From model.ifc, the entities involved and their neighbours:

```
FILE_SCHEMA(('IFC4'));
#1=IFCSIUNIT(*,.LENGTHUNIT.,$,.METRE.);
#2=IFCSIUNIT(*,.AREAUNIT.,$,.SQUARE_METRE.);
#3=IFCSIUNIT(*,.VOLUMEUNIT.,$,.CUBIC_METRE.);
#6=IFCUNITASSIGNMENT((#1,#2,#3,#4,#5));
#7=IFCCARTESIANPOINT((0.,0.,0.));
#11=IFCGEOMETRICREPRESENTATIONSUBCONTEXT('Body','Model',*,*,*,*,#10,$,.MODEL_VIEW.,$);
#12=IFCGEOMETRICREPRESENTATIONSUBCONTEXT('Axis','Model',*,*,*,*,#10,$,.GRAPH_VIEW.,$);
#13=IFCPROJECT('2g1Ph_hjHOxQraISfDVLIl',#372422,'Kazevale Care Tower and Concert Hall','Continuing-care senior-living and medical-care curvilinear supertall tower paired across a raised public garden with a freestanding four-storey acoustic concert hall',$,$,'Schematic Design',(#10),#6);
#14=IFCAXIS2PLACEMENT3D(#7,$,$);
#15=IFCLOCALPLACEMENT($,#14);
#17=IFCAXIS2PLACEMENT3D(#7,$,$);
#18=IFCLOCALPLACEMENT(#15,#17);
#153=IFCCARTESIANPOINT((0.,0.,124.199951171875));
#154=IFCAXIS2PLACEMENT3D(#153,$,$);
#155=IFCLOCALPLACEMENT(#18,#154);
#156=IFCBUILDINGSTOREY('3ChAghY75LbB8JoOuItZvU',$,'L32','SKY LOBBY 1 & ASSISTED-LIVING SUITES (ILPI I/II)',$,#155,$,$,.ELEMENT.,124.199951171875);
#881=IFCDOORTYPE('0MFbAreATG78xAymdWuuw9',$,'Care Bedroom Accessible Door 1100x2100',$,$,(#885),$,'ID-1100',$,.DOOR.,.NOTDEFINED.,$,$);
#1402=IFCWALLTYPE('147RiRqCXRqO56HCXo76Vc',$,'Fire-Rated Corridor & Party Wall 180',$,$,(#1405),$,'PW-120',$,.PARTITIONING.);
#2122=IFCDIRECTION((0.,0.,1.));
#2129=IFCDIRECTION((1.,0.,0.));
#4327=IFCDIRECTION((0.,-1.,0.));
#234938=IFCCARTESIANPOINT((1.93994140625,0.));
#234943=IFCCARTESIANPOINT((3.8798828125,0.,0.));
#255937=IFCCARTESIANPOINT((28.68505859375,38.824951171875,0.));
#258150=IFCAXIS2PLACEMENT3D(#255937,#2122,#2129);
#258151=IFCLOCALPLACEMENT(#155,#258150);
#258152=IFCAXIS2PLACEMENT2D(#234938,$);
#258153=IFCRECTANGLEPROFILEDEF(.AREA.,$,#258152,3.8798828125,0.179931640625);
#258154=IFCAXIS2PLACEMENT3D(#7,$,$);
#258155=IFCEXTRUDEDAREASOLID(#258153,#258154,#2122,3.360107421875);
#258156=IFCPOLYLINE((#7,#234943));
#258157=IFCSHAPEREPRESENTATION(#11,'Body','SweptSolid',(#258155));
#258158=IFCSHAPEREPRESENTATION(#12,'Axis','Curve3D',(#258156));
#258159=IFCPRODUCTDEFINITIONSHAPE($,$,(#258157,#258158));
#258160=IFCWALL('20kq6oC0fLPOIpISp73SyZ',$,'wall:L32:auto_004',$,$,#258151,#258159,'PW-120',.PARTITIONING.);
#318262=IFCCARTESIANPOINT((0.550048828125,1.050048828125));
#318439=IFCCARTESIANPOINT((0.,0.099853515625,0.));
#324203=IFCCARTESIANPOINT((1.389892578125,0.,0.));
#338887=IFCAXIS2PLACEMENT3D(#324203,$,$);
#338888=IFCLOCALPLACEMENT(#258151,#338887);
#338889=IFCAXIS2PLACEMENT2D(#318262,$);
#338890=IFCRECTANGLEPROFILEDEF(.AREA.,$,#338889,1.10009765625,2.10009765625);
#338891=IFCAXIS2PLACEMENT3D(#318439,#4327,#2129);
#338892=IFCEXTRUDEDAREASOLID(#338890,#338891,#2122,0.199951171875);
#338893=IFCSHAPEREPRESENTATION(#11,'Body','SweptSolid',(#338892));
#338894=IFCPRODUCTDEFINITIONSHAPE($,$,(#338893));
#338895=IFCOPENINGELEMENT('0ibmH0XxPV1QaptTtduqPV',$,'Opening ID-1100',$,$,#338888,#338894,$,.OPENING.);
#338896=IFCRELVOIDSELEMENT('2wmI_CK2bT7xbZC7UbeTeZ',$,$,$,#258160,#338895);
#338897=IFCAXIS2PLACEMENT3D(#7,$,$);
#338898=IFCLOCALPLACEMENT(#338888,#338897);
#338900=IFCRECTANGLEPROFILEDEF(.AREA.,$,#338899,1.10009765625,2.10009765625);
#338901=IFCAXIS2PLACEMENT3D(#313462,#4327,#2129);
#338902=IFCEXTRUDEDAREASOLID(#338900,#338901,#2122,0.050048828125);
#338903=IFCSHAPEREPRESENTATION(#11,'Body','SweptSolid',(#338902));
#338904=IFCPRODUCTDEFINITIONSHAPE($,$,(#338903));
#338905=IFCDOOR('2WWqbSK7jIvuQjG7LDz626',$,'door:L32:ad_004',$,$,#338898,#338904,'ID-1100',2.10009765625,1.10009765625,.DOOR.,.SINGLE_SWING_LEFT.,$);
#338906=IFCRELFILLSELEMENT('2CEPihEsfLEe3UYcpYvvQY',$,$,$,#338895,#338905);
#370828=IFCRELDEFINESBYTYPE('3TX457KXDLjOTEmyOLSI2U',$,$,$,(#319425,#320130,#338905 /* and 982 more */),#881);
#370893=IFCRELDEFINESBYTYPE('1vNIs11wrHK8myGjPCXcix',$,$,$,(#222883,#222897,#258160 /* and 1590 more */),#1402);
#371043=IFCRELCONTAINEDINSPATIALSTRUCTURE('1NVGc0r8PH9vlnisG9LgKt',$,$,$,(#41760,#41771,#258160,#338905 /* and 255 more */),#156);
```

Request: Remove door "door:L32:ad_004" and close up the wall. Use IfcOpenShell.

```python
import ifcopenshell
import ifcopenshell.api.feature
import ifcopenshell.api.root
import ifcopenshell.geom
import ifcopenshell.util.shape

model = ifcopenshell.open("model.ifc")
settings = ifcopenshell.geom.settings()


def volume(element):
    """Net volume in cubic metres, openings subtracted."""
    shape = ifcopenshell.geom.create_shape(settings, element)
    return ifcopenshell.util.shape.get_volume(shape.geometry)


door = model.by_guid("2WWqbSK7jIvuQjG7LDz626")
opening = door.FillsVoids[0].RelatingOpeningElement
wall = opening.VoidsElements[0].RelatingBuildingElement
before = volume(wall)

ifcopenshell.api.root.remove_product(model, product=door)
ifcopenshell.api.feature.remove_feature(model, feature=opening)

after = volume(wall)

print(f"wall volume {before:.3f} -> {after:.3f} m3")

model.write("model-out.ifc")
```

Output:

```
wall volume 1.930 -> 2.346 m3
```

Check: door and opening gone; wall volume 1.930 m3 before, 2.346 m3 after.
